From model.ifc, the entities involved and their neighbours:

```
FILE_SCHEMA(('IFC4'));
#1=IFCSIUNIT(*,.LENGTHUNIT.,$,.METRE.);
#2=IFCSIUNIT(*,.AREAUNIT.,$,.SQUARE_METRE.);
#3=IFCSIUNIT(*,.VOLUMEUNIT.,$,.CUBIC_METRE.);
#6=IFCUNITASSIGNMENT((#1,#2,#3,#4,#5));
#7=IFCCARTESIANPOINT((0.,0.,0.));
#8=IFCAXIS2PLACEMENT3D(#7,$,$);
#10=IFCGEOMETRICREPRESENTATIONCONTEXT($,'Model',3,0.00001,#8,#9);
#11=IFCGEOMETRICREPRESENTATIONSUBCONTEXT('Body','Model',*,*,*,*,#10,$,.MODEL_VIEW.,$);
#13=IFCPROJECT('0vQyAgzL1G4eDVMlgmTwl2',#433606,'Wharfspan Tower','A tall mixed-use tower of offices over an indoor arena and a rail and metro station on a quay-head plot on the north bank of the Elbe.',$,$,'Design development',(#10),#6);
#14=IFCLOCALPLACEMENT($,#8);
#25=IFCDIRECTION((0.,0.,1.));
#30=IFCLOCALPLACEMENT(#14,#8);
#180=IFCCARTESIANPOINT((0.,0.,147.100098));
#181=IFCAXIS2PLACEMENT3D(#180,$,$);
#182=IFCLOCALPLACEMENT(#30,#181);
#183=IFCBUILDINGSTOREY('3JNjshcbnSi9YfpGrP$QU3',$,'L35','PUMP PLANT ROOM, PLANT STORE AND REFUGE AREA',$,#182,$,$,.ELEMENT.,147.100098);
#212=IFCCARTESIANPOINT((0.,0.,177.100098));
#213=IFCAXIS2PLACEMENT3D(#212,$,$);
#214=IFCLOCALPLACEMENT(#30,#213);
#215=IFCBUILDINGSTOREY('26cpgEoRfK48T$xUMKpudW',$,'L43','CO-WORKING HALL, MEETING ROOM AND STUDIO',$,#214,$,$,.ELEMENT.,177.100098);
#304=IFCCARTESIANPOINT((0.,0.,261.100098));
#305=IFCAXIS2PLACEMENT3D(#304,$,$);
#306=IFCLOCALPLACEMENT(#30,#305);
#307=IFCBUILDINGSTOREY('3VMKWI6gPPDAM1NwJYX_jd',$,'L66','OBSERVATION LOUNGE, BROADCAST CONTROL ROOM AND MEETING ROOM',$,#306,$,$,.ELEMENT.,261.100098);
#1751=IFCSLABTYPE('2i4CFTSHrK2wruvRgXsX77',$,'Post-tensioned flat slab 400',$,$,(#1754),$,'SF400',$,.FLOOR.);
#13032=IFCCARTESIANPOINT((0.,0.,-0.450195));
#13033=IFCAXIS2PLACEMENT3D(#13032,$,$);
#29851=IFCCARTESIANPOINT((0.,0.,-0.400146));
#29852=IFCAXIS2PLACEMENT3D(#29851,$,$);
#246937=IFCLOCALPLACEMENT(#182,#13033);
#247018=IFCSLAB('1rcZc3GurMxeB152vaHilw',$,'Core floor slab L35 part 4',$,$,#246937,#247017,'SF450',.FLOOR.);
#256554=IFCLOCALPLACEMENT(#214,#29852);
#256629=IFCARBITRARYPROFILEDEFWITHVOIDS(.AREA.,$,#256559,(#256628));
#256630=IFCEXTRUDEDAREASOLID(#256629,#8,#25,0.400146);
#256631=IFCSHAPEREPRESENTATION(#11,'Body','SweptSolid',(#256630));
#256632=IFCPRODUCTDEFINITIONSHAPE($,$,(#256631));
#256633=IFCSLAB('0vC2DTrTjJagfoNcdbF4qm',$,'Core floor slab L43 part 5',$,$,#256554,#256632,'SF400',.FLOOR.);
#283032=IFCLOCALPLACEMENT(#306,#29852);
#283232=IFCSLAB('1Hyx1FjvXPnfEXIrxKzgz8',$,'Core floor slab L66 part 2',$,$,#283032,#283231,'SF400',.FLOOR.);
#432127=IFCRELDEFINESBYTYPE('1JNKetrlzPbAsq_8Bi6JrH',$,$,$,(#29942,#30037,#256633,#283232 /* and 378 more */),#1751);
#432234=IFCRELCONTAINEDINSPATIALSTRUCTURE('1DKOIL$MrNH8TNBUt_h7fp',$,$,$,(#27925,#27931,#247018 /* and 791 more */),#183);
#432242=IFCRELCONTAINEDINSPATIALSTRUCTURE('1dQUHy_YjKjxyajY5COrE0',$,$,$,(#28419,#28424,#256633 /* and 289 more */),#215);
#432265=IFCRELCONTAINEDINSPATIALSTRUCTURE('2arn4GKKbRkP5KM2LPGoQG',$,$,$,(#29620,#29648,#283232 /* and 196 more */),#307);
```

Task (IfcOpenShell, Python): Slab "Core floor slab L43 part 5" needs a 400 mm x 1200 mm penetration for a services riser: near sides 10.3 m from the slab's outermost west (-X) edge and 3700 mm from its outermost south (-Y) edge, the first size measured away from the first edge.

```python
import numpy as np
import ifcopenshell
import ifcopenshell.api.feature
import ifcopenshell.api.geometry
import ifcopenshell.api.root
import ifcopenshell.geom
import ifcopenshell.util.placement
import ifcopenshell.util.representation
import ifcopenshell.util.shape
import ifcopenshell.util.unit

model = ifcopenshell.open("model.ifc")
unit_scale = ifcopenshell.util.unit.calculate_unit_scale(model)
settings = ifcopenshell.geom.settings()


def volume(element):
    """Net volume in cubic metres, openings subtracted."""
    shape = ifcopenshell.geom.create_shape(settings, element)
    return ifcopenshell.util.shape.get_volume(shape.geometry)


slab = model.by_guid("0vC2DTrTjJagfoNcdbF4qm")
before = volume(slab)

# Extent in the slab's own axes, in metres. The edges named are its -X and -Y sides.
slab_shape = ifcopenshell.geom.create_shape(settings, slab)
vertices = ifcopenshell.util.shape.get_vertices(slab_shape.geometry)
x_min, y_min, bottom = vertices.min(axis=0)
top = vertices[:, 2].max()

opening = ifcopenshell.api.root.create_entity(model, ifc_class="IfcOpeningElement", name="Services riser opening", predefined_type="OPENING")
context = ifcopenshell.util.representation.get_context(model, "Model", "Body", "MODEL_VIEW")
width, depth = 0.4, 1.2
outline = [(0.0, 0.0), (width, 0.0), (width, depth), (0.0, depth), (0.0, 0.0)]
# Overshoot both faces by 50 mm so the cut is clean.
shape = ifcopenshell.api.geometry.add_slab_representation(
    model, context=context, depth=top - bottom + 0.1, polyline=outline
)
ifcopenshell.api.geometry.assign_representation(model, product=opening, representation=shape)

matrix = ifcopenshell.util.placement.get_local_placement(slab.ObjectPlacement)
matrix[:, 3] = matrix @ np.append(np.array([x_min + 10.3, y_min + 3.7, bottom - 0.05]) / unit_scale, 1.0)
ifcopenshell.api.geometry.edit_object_placement(model, product=opening, matrix=matrix, is_si=False)
ifcopenshell.api.feature.add_feature(model, feature=opening, element=slab)

after = volume(slab)

print(f"slab volume {before:.3f} -> {after:.3f} m3")

model.write("model_updated.ifc")
```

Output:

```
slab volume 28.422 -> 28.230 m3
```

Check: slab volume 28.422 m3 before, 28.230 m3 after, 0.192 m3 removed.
